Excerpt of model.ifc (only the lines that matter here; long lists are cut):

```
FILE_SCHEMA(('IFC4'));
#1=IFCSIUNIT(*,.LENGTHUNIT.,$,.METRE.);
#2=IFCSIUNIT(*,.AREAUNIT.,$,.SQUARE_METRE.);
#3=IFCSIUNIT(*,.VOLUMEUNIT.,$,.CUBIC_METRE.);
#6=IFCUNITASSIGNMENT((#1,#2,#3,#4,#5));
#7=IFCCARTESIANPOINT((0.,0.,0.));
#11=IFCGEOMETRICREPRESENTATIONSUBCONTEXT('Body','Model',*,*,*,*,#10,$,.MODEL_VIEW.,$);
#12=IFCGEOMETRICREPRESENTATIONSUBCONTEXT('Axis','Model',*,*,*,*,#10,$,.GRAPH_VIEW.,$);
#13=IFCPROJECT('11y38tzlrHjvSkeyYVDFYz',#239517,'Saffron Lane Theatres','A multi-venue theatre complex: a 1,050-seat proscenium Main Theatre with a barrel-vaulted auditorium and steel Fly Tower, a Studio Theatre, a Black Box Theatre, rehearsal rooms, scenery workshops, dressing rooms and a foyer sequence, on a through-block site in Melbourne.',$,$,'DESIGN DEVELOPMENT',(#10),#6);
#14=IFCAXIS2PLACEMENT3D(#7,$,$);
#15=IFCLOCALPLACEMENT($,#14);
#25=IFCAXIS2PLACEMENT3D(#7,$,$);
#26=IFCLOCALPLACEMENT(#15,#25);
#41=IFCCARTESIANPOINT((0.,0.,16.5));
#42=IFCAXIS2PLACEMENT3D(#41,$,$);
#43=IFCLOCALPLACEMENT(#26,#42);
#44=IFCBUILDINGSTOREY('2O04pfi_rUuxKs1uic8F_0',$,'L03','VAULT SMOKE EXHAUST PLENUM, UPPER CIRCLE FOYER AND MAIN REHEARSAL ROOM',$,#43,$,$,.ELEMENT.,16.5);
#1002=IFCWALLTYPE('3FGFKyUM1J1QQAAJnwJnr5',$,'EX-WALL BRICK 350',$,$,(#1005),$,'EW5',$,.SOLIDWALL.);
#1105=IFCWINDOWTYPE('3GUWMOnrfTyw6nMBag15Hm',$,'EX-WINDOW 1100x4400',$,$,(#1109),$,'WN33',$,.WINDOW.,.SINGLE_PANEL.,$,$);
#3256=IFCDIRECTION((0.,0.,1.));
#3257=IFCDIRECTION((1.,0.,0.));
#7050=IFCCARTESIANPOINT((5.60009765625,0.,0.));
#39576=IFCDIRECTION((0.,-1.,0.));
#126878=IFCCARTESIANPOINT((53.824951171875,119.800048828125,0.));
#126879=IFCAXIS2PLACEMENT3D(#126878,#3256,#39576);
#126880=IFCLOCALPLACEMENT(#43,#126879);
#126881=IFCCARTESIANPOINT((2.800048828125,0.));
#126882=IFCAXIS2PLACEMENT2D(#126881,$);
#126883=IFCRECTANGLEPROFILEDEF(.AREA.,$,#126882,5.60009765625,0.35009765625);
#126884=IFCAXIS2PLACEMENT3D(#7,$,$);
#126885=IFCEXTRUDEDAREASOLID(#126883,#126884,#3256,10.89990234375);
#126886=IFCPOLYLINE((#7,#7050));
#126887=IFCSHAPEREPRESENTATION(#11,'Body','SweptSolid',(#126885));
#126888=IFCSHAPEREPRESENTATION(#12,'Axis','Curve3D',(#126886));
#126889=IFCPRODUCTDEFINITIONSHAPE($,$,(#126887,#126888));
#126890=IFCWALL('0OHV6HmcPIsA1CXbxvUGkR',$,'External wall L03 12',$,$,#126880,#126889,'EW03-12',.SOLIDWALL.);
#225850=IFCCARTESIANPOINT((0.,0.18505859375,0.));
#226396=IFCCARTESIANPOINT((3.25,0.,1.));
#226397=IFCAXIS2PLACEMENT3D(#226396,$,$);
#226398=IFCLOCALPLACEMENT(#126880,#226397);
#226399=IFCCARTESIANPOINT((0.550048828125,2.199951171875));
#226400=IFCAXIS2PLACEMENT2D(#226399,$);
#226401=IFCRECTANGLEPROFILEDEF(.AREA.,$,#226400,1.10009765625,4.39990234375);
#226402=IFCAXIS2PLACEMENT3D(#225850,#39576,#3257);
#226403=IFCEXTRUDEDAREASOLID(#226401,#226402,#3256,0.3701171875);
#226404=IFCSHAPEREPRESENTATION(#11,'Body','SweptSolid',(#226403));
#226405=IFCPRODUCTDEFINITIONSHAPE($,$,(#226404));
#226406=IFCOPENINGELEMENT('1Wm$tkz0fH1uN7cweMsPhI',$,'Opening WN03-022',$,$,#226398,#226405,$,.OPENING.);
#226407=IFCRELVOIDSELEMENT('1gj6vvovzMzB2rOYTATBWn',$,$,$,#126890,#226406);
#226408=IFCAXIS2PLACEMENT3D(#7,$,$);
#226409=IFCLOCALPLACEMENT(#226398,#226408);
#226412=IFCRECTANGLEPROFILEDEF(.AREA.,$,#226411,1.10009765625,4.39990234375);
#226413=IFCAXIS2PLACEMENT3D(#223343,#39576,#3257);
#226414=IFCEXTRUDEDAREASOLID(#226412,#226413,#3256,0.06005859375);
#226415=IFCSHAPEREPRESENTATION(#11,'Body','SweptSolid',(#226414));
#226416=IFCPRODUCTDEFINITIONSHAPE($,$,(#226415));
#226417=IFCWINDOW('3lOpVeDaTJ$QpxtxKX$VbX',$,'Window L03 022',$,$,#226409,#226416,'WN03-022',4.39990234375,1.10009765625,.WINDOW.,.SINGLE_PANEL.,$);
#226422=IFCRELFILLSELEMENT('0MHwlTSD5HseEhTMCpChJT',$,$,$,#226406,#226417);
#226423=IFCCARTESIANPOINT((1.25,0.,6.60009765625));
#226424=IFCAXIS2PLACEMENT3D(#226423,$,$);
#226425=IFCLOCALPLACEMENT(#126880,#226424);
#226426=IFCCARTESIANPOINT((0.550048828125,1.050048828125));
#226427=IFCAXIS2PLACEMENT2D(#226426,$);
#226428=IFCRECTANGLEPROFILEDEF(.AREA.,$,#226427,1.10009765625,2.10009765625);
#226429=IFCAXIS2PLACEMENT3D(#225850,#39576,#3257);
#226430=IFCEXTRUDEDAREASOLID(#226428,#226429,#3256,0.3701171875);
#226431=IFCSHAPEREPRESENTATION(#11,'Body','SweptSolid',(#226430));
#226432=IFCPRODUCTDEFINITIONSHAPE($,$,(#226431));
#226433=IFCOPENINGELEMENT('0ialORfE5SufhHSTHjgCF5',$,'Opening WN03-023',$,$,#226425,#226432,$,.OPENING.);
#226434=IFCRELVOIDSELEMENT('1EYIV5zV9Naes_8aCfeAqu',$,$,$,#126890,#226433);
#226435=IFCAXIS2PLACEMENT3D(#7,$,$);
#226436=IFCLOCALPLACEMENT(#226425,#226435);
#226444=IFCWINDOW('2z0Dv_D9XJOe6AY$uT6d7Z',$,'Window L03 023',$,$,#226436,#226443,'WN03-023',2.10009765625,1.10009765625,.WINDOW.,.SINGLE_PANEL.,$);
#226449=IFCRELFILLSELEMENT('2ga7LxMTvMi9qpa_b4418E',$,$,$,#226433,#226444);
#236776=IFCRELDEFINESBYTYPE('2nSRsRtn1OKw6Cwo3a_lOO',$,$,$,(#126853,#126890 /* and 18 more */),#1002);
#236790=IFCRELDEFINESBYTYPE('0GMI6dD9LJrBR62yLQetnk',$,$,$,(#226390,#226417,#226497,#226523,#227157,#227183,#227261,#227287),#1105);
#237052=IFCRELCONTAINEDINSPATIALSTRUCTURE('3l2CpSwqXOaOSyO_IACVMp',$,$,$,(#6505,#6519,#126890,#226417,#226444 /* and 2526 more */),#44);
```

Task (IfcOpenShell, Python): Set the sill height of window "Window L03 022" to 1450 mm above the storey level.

```python
import numpy as np
import ifcopenshell
import ifcopenshell.api.geometry
import ifcopenshell.geom
import ifcopenshell.util.element
import ifcopenshell.util.placement
import ifcopenshell.util.shape
import ifcopenshell.util.unit

model = ifcopenshell.open("model.ifc")
unit_scale = ifcopenshell.util.unit.calculate_unit_scale(model)

window = model.by_id(226417)
opening = window.FillsVoids[0].RelatingOpeningElement
storey = ifcopenshell.util.element.get_container(window, ifc_class="IfcBuildingStorey")
level = ifcopenshell.util.placement.get_local_placement(storey.ObjectPlacement)[2, 3]

# The opening's origin need not be at the sill, so measure its lowest point.
shape = ifcopenshell.geom.create_shape(ifcopenshell.geom.settings(), opening)
bottom = ifcopenshell.util.shape.get_shape_bottom_elevation(shape, shape.geometry) / unit_scale
dz = level + 1.45 / unit_scale - bottom

shift = np.array([0.0, 0.0, dz])
# The window is placed relative to its opening, so it follows when the opening moves.
matrix = ifcopenshell.util.placement.get_local_placement(opening.ObjectPlacement)
matrix[:3, 3] += shift
ifcopenshell.api.geometry.edit_object_placement(
    model, product=opening, matrix=matrix, is_si=False, should_transform_children=True
)

print(f"moved by {dz * unit_scale:+.3f} m")

model.write("model_rev.ifc")
```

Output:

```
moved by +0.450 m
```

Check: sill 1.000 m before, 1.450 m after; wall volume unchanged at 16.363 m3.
